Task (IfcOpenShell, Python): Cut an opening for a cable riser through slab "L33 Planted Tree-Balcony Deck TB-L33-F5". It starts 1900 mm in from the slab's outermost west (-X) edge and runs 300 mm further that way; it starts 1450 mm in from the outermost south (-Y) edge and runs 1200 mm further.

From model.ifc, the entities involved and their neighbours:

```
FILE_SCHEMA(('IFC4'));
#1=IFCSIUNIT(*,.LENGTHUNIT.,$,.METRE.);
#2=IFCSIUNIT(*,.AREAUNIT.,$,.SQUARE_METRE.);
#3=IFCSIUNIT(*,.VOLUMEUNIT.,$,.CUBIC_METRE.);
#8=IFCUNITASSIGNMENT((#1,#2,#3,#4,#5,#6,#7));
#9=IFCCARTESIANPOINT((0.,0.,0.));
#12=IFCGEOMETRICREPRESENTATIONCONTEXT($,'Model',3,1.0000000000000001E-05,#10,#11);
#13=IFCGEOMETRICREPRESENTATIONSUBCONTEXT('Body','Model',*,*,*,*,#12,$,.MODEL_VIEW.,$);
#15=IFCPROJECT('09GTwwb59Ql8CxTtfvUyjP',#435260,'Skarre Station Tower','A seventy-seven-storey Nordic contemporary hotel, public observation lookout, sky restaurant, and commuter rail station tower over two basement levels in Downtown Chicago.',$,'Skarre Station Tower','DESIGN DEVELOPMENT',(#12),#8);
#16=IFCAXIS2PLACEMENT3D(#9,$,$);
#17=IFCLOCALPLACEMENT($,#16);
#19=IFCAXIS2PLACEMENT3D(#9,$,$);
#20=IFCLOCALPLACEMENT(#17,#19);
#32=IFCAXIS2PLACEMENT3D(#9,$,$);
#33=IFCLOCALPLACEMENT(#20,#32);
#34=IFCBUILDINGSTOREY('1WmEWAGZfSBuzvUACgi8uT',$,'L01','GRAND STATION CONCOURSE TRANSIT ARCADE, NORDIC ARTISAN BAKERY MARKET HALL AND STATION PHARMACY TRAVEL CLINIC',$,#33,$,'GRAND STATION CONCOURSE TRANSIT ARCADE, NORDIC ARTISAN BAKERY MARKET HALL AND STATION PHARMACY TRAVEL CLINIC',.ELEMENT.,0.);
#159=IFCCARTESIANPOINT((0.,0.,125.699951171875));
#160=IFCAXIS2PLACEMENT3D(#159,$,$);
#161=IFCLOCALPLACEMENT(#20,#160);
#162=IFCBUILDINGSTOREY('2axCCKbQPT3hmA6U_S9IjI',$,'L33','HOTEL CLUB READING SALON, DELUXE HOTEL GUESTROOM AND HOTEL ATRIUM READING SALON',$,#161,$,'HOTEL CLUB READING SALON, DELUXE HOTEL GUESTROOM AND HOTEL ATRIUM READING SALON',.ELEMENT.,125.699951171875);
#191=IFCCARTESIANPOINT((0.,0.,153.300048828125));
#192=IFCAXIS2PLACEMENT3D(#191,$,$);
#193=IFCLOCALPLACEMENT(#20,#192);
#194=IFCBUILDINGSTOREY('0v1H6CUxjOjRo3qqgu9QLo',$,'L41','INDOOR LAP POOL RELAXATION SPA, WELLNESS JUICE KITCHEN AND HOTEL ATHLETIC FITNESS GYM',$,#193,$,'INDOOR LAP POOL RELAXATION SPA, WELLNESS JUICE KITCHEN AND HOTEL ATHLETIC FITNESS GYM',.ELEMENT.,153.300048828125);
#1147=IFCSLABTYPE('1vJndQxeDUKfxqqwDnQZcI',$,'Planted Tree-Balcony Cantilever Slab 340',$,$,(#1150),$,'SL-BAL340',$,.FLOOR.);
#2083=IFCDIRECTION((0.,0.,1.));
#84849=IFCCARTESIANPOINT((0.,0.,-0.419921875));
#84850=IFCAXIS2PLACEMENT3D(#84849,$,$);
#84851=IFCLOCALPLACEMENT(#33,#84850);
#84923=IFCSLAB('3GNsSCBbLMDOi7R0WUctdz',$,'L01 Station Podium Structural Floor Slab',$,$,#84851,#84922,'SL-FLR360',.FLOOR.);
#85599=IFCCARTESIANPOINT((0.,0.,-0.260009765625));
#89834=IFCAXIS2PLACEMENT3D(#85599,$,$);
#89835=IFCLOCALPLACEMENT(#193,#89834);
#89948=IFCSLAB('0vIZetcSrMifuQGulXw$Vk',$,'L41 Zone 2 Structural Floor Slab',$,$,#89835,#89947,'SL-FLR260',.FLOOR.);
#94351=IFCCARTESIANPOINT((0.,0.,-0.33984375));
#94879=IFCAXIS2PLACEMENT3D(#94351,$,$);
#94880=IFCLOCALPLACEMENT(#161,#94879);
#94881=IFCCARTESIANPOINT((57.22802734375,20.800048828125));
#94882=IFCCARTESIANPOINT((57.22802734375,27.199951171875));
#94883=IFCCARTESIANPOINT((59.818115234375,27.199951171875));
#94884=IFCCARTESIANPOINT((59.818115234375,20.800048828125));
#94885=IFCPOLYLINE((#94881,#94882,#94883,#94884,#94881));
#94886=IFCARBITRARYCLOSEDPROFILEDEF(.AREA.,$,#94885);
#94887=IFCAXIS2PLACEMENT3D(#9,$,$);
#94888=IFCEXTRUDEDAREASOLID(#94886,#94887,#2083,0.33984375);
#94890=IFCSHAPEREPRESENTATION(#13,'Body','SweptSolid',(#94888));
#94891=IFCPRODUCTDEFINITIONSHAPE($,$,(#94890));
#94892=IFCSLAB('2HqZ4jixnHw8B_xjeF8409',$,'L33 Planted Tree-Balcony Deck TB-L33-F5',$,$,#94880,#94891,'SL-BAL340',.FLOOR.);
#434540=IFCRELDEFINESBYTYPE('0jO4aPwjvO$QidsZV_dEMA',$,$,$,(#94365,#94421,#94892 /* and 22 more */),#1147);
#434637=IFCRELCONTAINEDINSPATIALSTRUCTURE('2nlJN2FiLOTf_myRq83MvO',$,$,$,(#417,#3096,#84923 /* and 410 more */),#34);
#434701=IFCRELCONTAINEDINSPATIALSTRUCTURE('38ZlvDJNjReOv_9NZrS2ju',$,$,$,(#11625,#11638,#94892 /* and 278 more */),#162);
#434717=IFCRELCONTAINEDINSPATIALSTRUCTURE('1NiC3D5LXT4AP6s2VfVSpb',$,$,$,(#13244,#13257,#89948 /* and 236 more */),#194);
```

```python
import numpy as np
import ifcopenshell
import ifcopenshell.api.feature
import ifcopenshell.api.geometry
import ifcopenshell.api.root
import ifcopenshell.geom
import ifcopenshell.util.placement
import ifcopenshell.util.representation
import ifcopenshell.util.shape
import ifcopenshell.util.unit

model = ifcopenshell.open("model.ifc")
unit_scale = ifcopenshell.util.unit.calculate_unit_scale(model)
settings = ifcopenshell.geom.settings()


def volume(element):
    """Net volume in cubic metres, openings subtracted."""
    shape = ifcopenshell.geom.create_shape(settings, element)
    return ifcopenshell.util.shape.get_volume(shape.geometry)


slab = model.by_guid("2HqZ4jixnHw8B_xjeF8409")
before = volume(slab)

# Extent in the slab's own axes, in metres. The edges named are its -X and -Y sides.
slab_shape = ifcopenshell.geom.create_shape(settings, slab)
vertices = ifcopenshell.util.shape.get_vertices(slab_shape.geometry)
x_min, y_min, bottom = vertices.min(axis=0)
top = vertices[:, 2].max()

opening = ifcopenshell.api.root.create_entity(model, ifc_class="IfcOpeningElement", name="Cable riser opening", predefined_type="OPENING")
context = ifcopenshell.util.representation.get_context(model, "Model", "Body", "MODEL_VIEW")
width, depth = 0.3, 1.2
outline = [(0.0, 0.0), (width, 0.0), (width, depth), (0.0, depth), (0.0, 0.0)]
# Overshoot both faces by 50 mm so the cut is clean.
shape = ifcopenshell.api.geometry.add_slab_representation(
    model, context=context, depth=top - bottom + 0.1, polyline=outline
)
ifcopenshell.api.geometry.assign_representation(model, product=opening, representation=shape)

matrix = ifcopenshell.util.placement.get_local_placement(slab.ObjectPlacement)
matrix[:, 3] = matrix @ np.append(np.array([x_min + 1.9, y_min + 1.45, bottom - 0.05]) / unit_scale, 1.0)
ifcopenshell.api.geometry.edit_object_placement(model, product=opening, matrix=matrix, is_si=False)
ifcopenshell.api.feature.add_feature(model, feature=opening, element=slab)

after = volume(slab)

print(f"slab volume {before:.3f} -> {after:.3f} m3")

model.write("model_edited.ifc")
```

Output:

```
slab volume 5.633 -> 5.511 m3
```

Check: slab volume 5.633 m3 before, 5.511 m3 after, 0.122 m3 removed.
